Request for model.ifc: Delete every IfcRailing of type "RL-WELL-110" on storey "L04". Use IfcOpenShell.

First a look at what the model holds.

```python
import ifcopenshell
import ifcopenshell.util.element

model = ifcopenshell.open("model.ifc")
print(model.schema)
storey = next(s for s in model.by_type("IfcBuildingStorey") if s.Name == "L04")
railings = [e for e in ifcopenshell.util.element.get_decomposition(storey) if e.is_a("IfcRailing")]
seen = {}
for e in railings:
    element_type = ifcopenshell.util.element.get_type(e)
    name = element_type.Name if element_type not in (None, e) else None
    seen[name] = seen.get(name, 0) + 1
for name, count in sorted(seen.items(), key=str):
    print(count, "x", name)
```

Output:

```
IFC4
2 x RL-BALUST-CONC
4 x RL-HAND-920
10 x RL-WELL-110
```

```python
import ifcopenshell
import ifcopenshell.api.root
import ifcopenshell.util.element

model = ifcopenshell.open("model.ifc")

storey = next(s for s in model.by_type("IfcBuildingStorey") if s.Name == "L04")
railings = [e for e in ifcopenshell.util.element.get_decomposition(storey) if e.is_a("IfcRailing")]
targets = [e for e in railings if (t := ifcopenshell.util.element.get_type(e)) not in (None, e) and t.Name == "RL-WELL-110"]

for e in targets:
    ifcopenshell.api.root.remove_product(model, product=e)
print(len(targets), "removed")

model.write("model_edited.ifc")
```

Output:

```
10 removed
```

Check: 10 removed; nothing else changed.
